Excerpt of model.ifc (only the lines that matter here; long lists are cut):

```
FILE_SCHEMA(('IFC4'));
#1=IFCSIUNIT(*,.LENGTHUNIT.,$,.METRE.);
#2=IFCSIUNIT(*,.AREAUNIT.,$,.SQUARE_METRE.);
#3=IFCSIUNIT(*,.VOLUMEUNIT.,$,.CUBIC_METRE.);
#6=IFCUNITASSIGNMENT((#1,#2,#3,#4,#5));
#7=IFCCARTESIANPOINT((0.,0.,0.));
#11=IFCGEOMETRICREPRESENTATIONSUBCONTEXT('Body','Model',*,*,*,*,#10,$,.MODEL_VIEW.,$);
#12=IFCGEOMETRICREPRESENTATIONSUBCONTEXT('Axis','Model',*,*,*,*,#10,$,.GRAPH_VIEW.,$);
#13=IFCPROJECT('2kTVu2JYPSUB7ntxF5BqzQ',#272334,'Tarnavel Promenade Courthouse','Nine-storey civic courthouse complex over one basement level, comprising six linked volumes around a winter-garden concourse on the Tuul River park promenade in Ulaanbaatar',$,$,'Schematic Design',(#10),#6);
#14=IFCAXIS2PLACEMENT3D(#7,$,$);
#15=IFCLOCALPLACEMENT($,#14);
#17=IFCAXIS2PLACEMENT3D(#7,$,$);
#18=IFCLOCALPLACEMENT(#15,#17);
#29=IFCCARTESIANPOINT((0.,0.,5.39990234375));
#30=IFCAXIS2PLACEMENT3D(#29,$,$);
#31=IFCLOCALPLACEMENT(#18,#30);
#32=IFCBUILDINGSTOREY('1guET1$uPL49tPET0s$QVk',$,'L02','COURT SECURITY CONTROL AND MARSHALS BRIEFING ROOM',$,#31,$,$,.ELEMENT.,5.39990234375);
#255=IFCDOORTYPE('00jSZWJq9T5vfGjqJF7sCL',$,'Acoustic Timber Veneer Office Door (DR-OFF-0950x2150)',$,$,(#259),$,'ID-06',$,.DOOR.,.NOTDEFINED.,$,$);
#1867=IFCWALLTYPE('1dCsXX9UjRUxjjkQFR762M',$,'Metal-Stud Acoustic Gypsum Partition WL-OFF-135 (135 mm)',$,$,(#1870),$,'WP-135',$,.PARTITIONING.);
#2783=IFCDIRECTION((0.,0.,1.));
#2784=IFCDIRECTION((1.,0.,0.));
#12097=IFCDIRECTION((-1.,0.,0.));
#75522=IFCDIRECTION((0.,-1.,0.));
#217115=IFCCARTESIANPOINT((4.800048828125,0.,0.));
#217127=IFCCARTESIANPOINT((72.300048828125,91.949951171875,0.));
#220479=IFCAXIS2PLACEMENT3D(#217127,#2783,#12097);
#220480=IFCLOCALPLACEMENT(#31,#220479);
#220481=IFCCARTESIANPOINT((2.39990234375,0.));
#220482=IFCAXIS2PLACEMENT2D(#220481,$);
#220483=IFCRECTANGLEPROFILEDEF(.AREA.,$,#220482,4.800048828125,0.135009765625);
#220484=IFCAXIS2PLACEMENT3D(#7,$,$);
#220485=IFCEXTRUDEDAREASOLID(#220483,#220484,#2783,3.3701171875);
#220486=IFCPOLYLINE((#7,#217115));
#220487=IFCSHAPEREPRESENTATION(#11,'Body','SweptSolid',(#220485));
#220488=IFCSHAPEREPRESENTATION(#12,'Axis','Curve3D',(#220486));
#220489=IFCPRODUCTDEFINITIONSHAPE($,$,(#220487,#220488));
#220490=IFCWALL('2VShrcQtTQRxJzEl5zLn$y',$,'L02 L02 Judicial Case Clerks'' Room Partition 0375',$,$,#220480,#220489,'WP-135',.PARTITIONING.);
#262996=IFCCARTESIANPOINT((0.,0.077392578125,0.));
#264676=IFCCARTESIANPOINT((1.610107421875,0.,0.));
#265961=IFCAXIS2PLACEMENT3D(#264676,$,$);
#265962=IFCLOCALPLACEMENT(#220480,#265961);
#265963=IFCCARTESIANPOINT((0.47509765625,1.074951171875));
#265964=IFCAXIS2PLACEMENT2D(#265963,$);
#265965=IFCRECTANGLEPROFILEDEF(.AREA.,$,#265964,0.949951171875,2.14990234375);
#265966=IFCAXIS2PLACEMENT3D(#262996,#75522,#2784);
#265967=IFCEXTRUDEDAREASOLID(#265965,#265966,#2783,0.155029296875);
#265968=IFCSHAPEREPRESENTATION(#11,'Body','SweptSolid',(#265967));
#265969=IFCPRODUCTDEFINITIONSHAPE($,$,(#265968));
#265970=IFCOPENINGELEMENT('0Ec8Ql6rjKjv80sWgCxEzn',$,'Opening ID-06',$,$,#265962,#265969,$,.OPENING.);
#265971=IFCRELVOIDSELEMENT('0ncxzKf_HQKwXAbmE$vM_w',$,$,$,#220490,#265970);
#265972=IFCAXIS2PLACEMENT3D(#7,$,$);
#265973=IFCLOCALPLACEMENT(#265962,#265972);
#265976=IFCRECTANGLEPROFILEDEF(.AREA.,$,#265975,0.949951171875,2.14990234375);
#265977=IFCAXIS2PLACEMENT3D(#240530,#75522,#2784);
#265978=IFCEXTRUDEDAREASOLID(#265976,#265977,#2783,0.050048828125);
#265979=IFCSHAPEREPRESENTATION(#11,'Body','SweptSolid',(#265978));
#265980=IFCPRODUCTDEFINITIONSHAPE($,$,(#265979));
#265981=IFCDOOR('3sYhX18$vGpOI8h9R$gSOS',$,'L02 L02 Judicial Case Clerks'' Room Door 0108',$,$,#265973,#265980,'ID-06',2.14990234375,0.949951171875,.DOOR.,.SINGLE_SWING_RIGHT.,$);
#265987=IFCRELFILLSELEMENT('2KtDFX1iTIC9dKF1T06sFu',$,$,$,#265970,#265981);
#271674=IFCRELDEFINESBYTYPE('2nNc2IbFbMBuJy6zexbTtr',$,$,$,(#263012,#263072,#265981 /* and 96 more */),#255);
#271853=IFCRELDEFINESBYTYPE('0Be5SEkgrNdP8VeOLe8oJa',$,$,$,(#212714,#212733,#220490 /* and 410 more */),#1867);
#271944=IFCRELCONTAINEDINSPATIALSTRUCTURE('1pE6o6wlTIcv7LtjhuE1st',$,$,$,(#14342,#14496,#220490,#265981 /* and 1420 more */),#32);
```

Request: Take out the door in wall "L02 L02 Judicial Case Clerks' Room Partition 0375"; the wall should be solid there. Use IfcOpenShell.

```python
import ifcopenshell
import ifcopenshell.api.feature
import ifcopenshell.api.root
import ifcopenshell.geom
import ifcopenshell.util.shape

model = ifcopenshell.open("model.ifc")
settings = ifcopenshell.geom.settings()


def volume(element):
    """Net volume in cubic metres, openings subtracted."""
    shape = ifcopenshell.geom.create_shape(settings, element)
    return ifcopenshell.util.shape.get_volume(shape.geometry)


door = model.by_guid("3sYhX18$vGpOI8h9R$gSOS")
opening = door.FillsVoids[0].RelatingOpeningElement
wall = opening.VoidsElements[0].RelatingBuildingElement
before = volume(wall)

ifcopenshell.api.root.remove_product(model, product=door)
ifcopenshell.api.feature.remove_feature(model, feature=opening)

after = volume(wall)

print(f"wall volume {before:.3f} -> {after:.3f} m3")

model.write("model_rev.ifc")
```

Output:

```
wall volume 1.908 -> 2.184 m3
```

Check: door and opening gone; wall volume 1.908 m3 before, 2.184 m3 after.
